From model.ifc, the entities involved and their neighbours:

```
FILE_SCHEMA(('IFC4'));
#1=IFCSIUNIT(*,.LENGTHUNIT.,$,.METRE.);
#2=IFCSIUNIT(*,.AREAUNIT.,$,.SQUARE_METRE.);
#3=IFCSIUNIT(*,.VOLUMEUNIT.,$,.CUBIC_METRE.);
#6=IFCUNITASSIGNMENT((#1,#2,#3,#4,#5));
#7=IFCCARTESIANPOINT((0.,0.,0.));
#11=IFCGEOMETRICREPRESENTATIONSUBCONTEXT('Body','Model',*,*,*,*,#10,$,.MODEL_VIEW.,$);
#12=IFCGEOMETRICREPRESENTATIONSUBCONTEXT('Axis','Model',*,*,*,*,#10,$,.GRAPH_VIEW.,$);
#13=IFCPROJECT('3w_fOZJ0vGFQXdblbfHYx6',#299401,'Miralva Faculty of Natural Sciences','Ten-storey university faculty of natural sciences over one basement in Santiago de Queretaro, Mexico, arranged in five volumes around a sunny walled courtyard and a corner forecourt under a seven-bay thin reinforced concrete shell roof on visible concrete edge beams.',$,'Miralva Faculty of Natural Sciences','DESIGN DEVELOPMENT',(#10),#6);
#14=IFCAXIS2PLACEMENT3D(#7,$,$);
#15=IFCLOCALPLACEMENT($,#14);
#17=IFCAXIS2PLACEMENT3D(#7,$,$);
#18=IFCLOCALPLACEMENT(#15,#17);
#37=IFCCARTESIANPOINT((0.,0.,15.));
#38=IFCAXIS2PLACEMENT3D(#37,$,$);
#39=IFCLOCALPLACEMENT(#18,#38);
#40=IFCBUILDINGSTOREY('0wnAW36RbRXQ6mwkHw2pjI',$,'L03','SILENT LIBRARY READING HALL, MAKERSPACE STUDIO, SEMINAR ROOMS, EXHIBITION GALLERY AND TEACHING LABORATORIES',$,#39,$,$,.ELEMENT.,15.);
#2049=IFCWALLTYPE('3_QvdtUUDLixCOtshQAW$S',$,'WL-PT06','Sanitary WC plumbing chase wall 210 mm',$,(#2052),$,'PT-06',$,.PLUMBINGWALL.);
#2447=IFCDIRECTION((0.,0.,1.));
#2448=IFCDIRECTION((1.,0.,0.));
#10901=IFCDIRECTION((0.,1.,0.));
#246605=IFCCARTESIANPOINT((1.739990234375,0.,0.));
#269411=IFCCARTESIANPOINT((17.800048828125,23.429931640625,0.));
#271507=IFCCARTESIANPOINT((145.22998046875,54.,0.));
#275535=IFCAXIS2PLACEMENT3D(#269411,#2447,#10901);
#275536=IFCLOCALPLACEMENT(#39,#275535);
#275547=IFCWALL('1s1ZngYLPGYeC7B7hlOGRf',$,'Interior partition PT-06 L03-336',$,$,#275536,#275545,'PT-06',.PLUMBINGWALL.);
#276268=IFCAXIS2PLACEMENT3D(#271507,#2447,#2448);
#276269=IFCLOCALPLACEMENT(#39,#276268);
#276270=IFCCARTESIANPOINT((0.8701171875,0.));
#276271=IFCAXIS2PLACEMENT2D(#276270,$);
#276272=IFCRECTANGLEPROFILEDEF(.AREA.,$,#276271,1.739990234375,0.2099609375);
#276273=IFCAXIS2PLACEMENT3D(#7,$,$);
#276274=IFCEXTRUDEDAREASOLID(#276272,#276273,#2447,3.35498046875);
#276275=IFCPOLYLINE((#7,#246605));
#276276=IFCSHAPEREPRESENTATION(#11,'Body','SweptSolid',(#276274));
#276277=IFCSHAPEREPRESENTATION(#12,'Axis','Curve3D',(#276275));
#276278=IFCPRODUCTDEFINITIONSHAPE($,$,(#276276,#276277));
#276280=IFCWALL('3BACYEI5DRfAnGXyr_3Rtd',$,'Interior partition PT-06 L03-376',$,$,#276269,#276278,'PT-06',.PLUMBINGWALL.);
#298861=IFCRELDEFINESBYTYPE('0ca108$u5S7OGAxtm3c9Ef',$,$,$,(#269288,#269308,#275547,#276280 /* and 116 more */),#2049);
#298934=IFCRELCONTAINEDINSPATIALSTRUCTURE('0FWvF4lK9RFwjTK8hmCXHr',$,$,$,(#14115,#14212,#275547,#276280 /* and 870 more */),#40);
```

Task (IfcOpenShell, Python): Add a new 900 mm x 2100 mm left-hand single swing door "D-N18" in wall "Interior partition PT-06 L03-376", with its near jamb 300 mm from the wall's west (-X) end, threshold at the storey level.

```python
import numpy as np
import ifcopenshell
import ifcopenshell.api.feature
import ifcopenshell.api.geometry
import ifcopenshell.api.root
import ifcopenshell.api.spatial
import ifcopenshell.geom
import ifcopenshell.util.element
import ifcopenshell.util.placement
import ifcopenshell.util.representation
import ifcopenshell.util.shape
import ifcopenshell.util.unit

model = ifcopenshell.open("model.ifc")
unit_scale = ifcopenshell.util.unit.calculate_unit_scale(model)
settings = ifcopenshell.geom.settings()


def volume(element):
    """Net volume in cubic metres, openings subtracted."""
    shape = ifcopenshell.geom.create_shape(settings, element)
    return ifcopenshell.util.shape.get_volume(shape.geometry)


wall = model.by_guid("3BACYEI5DRfAnGXyr_3Rtd")
storey = ifcopenshell.util.element.get_container(wall, ifc_class="IfcBuildingStorey")
context = ifcopenshell.util.representation.get_context(model, "Model", "Body", "MODEL_VIEW")
before = volume(wall)

width, height, from_end, sill = 0.9, 2.1, 0.3, 0.0  # metres

# The wall runs along its own X axis, and the end named is its -X end.
wall_shape = ifcopenshell.geom.create_shape(settings, wall)
x, y, z = ifcopenshell.util.shape.get_vertices(wall_shape.geometry).T
start = x.min() + from_end
face, thickness = float(y.min()), float(y.max() - y.min())
wall_matrix = ifcopenshell.util.placement.get_local_placement(wall.ObjectPlacement)
level = ifcopenshell.util.placement.get_local_placement(storey.ObjectPlacement)[2, 3]


def in_wall(x, y):
    """Placement at x, y metres in the wall's axes, at sill height."""
    matrix = wall_matrix.copy()
    matrix[:, 3] = wall_matrix @ np.array([x / unit_scale, y / unit_scale, 0.0, 1.0])
    matrix[2, 3] = level + sill / unit_scale
    return matrix


# Opening: a box that overshoots both wall faces by 50 mm.
opening = ifcopenshell.api.root.create_entity(model, ifc_class="IfcOpeningElement", predefined_type="OPENING")
box = ifcopenshell.api.geometry.add_wall_representation(
    model, context=context, length=width, height=height, thickness=thickness + 0.1
)
ifcopenshell.api.geometry.assign_representation(model, product=opening, representation=box)
ifcopenshell.api.geometry.edit_object_placement(model, product=opening, matrix=in_wall(start, face - 0.05), is_si=False)
ifcopenshell.api.feature.add_feature(model, feature=opening, element=wall)

door = ifcopenshell.api.root.create_entity(model, ifc_class="IfcDoor", name="D-N18", predefined_type="DOOR")
door.OverallWidth, door.OverallHeight = width / unit_scale, height / unit_scale
door.OperationType = "SINGLE_SWING_LEFT"
body = ifcopenshell.api.geometry.add_door_representation(
    model,
    context=context,
    overall_width=door.OverallWidth,
    overall_height=door.OverallHeight,
    operation_type="SINGLE_SWING_LEFT",
    lining_properties={"LiningDepth": thickness / unit_scale, "ThresholdDepth": thickness / unit_scale},
)
ifcopenshell.api.geometry.assign_representation(model, product=door, representation=body)
ifcopenshell.api.spatial.assign_container(model, products=[door], relating_structure=storey)
ifcopenshell.api.feature.add_filling(model, opening=opening, element=door)

# The lining spans the wall, so the door starts at the wall face.
ifcopenshell.api.geometry.edit_object_placement(model, product=door, matrix=in_wall(start, face), is_si=False)

after = volume(wall)

print(f"wall volume {before:.3f} -> {after:.3f} m3")

model.write("model-out.ifc")
```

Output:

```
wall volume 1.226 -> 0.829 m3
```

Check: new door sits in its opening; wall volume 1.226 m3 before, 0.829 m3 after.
